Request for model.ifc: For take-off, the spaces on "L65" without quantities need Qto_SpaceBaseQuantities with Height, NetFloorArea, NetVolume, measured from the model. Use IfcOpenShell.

First a look at what the model holds.

```python
import ifcopenshell
import ifcopenshell.util.element
import ifcopenshell.util.unit

model = ifcopenshell.open("model.ifc")
print(model.schema)
for unit_type in ("LENGTHUNIT", "AREAUNIT", "VOLUMEUNIT"):
    print(unit_type, ifcopenshell.util.unit.calculate_unit_scale(model, unit_type))
storey = next(s for s in model.by_type("IfcBuildingStorey") if s.Name == "L65")
spaces = [e for e in ifcopenshell.util.element.get_decomposition(storey) if e.is_a("IfcSpace")]
for e in sorted(spaces, key=lambda e: e.id()):
    print(e.id(), e.is_a(), e.Name, list(ifcopenshell.util.element.get_psets(e, qtos_only=True)), sep=" | ")
```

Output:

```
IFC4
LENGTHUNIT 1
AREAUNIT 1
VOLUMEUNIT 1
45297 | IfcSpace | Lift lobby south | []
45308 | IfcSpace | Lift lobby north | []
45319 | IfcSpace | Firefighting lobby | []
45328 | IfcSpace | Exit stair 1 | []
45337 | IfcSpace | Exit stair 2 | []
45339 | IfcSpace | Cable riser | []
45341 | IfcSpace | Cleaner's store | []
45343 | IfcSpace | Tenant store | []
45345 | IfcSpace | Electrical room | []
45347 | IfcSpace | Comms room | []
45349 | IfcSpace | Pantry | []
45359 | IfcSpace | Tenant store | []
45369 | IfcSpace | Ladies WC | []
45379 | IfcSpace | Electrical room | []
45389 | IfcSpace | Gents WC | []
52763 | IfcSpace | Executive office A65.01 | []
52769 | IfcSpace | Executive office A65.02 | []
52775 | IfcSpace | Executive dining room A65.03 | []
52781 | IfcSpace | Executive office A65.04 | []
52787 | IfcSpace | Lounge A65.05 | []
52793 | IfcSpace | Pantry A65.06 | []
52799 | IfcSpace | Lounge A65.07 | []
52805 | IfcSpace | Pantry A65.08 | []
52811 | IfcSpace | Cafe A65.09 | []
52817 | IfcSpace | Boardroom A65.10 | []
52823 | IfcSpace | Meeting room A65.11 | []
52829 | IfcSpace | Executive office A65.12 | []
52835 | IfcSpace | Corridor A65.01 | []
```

```python
import ifcopenshell
import ifcopenshell.api.pset
import ifcopenshell.geom
import ifcopenshell.util.element
import ifcopenshell.util.shape
import ifcopenshell.util.unit

model = ifcopenshell.open("model.ifc")
unit_scale = ifcopenshell.util.unit.calculate_unit_scale(model)
area_scale = ifcopenshell.util.unit.calculate_unit_scale(model, "AREAUNIT")
volume_scale = ifcopenshell.util.unit.calculate_unit_scale(model, "VOLUMEUNIT")
settings = ifcopenshell.geom.settings()

storey = next(s for s in model.by_type("IfcBuildingStorey") if s.Name == "L65")
spaces = [e for e in ifcopenshell.util.element.get_decomposition(storey) if e.is_a("IfcSpace")]

for e in sorted(spaces, key=lambda e: e.id()):
    if ifcopenshell.util.element.get_psets(e, qtos_only=True, should_inherit=False):
        continue
    # Geometry comes back in metres, in the element's own axes.
    shape = ifcopenshell.geom.create_shape(settings, e)
    values = {
        "Height": ifcopenshell.util.shape.get_z(shape.geometry) / unit_scale,
        "NetFloorArea": ifcopenshell.util.shape.get_footprint_area(shape.geometry) / area_scale,
        "NetVolume": ifcopenshell.util.shape.get_volume(shape.geometry) / volume_scale,
    }
    qto = ifcopenshell.api.pset.add_qto(model, product=e, name="Qto_SpaceBaseQuantities")
    ifcopenshell.api.pset.edit_qto(model, qto=qto, properties=values)
    print(e.id(), {k: round(v, 3) for k, v in values.items()})

model.write("model_v2.ifc")
```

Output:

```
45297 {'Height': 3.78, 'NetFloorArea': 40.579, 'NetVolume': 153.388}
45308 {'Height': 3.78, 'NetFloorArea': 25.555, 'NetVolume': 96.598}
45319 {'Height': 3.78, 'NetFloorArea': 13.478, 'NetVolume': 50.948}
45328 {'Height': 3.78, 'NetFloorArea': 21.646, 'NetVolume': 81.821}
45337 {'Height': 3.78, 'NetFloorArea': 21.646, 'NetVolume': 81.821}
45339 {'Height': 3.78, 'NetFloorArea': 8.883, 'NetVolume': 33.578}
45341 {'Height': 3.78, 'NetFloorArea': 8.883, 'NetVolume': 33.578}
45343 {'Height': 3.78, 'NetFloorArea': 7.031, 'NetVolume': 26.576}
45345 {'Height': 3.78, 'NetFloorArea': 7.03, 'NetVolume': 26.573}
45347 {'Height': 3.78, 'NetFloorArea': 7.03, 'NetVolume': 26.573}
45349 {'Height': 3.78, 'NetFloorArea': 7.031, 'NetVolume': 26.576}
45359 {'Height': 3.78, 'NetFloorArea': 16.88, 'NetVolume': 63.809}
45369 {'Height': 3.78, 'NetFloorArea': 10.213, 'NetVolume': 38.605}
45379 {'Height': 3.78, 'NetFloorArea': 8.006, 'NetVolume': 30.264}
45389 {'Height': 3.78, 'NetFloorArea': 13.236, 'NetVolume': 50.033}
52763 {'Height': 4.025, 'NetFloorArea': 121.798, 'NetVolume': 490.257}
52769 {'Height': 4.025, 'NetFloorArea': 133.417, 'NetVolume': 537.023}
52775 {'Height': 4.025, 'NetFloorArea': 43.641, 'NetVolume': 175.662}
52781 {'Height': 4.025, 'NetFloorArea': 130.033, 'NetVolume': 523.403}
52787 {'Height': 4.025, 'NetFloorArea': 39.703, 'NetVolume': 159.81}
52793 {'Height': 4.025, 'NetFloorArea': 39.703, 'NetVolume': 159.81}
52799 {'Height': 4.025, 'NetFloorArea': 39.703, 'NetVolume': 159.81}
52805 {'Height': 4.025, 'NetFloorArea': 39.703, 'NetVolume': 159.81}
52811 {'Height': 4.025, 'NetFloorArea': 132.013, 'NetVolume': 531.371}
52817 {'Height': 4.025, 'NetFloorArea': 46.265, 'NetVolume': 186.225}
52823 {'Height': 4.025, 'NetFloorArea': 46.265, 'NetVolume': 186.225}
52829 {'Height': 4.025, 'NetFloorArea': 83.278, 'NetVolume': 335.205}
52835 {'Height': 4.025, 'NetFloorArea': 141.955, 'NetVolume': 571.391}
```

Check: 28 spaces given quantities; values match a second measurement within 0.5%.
